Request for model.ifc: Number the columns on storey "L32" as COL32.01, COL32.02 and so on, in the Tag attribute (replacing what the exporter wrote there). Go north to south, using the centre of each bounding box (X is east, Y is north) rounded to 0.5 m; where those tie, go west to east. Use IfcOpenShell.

First a look at what the model holds.

```python
import ifcopenshell
import ifcopenshell.util.element
import ifcopenshell.util.placement

model = ifcopenshell.open("model.ifc")
print(model.schema)
storey = next(s for s in model.by_type("IfcBuildingStorey") if s.Name == "L32")
columns = [e for e in ifcopenshell.util.element.get_decomposition(storey) if e.is_a("IfcColumn")]
for e in sorted(columns, key=lambda e: e.id()):
    origin = ifcopenshell.util.placement.get_local_placement(e.ObjectPlacement)[:3, 3]
    print(e.id(), e.Tag, e.Name, origin.round(2) + 0.0, sep=" | ")
```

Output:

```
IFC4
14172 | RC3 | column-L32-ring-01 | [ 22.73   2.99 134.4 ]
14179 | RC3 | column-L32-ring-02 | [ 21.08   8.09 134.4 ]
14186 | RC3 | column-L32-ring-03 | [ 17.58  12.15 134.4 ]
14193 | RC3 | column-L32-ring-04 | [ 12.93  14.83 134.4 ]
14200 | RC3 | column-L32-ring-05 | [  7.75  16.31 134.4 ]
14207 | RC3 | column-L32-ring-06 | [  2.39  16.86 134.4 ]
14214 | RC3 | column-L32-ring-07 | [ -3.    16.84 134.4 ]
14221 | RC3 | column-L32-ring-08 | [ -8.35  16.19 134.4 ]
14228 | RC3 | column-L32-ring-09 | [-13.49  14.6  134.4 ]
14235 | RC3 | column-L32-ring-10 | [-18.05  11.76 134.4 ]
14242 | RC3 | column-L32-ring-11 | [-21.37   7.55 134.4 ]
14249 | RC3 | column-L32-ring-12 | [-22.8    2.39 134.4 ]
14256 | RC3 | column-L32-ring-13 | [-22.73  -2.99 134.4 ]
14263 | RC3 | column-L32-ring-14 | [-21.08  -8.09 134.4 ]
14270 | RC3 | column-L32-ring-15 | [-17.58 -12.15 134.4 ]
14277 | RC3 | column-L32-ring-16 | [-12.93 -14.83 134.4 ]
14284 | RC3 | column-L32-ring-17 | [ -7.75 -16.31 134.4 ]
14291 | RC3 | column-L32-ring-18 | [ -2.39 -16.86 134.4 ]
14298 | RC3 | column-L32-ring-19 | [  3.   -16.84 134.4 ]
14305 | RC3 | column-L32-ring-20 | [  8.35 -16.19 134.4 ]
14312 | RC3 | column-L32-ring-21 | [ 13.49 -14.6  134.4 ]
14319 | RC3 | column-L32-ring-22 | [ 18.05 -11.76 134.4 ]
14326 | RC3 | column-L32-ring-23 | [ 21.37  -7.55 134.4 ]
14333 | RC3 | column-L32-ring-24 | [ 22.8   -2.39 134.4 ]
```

```python
import ifcopenshell
import ifcopenshell.geom
import ifcopenshell.util.element
import ifcopenshell.util.shape

model = ifcopenshell.open("model.ifc")
settings = ifcopenshell.geom.settings()
settings.set("use-world-coords", True)


def centre(element):
    shape = ifcopenshell.geom.create_shape(settings, element)
    return ifcopenshell.util.shape.get_bbox_centroid(shape.geometry)


storey = next(s for s in model.by_type("IfcBuildingStorey") if s.Name == "L32")
columns = [e for e in ifcopenshell.util.element.get_decomposition(storey) if e.is_a("IfcColumn")]

# Insertion points can sit at a corner or the storey origin, so sort by the geometry (in metres).
centres = {e: centre(e) for e in columns}
columns.sort(key=lambda e: (-round(centres[e][1] / 0.5), centres[e][0]))

for i, e in enumerate(columns, start=1):
    number = f"COL32.{i:02d}"
    e.Tag = number
    print(e.id(), number)

model.write("model_v2.ifc")
```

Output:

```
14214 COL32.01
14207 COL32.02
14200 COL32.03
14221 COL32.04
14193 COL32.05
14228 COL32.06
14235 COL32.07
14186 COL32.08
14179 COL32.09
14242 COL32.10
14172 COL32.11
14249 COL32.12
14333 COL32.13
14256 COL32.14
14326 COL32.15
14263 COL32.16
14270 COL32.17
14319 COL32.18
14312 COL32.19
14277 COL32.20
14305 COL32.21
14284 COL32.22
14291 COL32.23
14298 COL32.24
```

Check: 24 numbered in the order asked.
